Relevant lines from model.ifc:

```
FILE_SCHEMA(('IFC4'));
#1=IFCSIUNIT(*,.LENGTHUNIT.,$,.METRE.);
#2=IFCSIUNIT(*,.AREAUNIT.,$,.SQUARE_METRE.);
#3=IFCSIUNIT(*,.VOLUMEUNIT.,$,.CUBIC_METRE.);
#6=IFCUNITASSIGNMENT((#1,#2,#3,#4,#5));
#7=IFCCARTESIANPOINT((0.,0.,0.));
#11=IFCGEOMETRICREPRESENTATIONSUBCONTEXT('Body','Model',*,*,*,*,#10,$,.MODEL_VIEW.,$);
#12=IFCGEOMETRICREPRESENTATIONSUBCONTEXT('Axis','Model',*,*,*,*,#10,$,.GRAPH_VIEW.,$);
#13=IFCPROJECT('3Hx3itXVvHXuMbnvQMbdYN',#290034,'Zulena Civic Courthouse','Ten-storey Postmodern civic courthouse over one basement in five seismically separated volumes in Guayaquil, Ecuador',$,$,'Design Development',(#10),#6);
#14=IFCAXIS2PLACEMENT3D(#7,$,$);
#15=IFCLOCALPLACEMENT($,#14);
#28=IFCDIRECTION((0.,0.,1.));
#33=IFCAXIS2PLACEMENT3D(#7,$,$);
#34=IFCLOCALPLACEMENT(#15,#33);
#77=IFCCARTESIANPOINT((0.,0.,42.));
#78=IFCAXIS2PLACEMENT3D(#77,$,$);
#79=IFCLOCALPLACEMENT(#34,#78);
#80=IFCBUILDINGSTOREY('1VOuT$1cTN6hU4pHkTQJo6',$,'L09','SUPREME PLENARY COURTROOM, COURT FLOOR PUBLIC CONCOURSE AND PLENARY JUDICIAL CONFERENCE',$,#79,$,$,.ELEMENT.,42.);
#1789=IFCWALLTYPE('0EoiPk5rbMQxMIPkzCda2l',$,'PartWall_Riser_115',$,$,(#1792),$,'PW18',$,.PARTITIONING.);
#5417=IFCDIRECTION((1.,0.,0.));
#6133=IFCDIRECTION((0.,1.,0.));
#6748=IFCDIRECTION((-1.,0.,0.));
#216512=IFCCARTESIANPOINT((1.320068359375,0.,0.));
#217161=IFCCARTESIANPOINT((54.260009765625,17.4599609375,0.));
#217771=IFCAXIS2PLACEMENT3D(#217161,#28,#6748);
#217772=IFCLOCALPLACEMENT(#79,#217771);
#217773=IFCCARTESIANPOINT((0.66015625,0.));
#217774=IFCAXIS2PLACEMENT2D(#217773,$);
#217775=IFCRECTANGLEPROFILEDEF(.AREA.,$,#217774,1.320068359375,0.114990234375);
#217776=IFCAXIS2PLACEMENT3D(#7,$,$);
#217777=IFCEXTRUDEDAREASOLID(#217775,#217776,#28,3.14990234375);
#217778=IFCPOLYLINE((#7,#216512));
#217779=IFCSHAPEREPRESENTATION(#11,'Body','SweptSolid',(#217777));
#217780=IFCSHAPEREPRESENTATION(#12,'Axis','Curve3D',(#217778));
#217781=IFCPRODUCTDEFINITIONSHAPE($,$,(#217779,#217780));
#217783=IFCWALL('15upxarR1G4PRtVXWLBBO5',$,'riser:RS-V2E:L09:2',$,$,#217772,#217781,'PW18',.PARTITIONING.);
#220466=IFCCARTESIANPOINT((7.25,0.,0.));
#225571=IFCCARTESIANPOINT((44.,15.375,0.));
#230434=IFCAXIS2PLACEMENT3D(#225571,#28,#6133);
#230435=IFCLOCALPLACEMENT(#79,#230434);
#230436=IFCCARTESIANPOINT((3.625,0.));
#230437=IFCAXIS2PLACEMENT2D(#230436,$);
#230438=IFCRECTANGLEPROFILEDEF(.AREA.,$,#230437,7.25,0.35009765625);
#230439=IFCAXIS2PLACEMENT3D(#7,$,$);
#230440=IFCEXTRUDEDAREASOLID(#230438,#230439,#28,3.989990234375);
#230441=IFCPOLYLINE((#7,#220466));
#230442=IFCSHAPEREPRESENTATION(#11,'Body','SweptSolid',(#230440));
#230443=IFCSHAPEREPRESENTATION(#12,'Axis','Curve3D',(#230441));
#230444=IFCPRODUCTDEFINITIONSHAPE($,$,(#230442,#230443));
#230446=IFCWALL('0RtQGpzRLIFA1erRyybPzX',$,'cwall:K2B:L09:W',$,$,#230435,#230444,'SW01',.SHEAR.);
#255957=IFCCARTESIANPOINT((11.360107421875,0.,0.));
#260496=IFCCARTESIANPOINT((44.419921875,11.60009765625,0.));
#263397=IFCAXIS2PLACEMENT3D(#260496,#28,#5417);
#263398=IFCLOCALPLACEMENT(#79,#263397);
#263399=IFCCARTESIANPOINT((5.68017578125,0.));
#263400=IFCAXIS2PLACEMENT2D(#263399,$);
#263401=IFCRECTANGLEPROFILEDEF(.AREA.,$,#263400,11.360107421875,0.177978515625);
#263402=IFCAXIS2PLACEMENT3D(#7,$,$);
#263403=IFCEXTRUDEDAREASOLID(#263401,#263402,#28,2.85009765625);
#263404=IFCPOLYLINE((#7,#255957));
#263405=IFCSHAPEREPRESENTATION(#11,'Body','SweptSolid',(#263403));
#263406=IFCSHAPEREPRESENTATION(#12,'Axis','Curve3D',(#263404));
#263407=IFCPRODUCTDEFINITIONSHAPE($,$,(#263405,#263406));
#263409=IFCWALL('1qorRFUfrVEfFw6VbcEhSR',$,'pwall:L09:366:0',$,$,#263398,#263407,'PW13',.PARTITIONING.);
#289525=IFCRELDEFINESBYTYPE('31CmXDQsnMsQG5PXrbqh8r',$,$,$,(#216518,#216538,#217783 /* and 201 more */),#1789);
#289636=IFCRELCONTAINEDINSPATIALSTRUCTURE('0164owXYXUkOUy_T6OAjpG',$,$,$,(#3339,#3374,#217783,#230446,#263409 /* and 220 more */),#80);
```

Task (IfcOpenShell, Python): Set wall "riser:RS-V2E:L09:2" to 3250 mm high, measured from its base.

```python
import ifcopenshell
import ifcopenshell.geom
import ifcopenshell.util.representation
import ifcopenshell.util.shape
import ifcopenshell.util.unit

model = ifcopenshell.open("model.ifc")
unit_scale = ifcopenshell.util.unit.calculate_unit_scale(model)
settings = ifcopenshell.geom.settings()


def volume(element):
    """Net volume in cubic metres, openings subtracted."""
    shape = ifcopenshell.geom.create_shape(settings, element)
    return ifcopenshell.util.shape.get_volume(shape.geometry)


wall = model.by_guid("15upxarR1G4PRtVXWLBBO5")
before = volume(wall)

body = ifcopenshell.util.representation.get_representation(wall, "Model", "Body")
solid = body.Items[0]
old_height = solid.Depth
solid.Depth = 3.25 / unit_scale
after = volume(wall)

print(f"height {old_height:g} -> {solid.Depth:g}, volume {before:.3f} -> {after:.3f} m3")

model.write("model_rev.ifc")
```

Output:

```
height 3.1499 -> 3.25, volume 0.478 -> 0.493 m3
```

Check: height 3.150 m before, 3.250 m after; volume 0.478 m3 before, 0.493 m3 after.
